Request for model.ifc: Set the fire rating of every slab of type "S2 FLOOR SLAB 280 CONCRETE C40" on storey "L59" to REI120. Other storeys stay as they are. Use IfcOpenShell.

First a look at what the model holds.

```python
import ifcopenshell
import ifcopenshell.util.element

model = ifcopenshell.open("model.ifc")
print(model.schema)
storey = next(s for s in model.by_type("IfcBuildingStorey") if s.Name == "L59")
slabs = [e for e in ifcopenshell.util.element.get_decomposition(storey) if e.is_a("IfcSlab")]
seen = {}
for e in slabs:
    element_type = ifcopenshell.util.element.get_type(e)
    key = (element_type.Name if element_type != e and element_type else None, ifcopenshell.util.element.get_pset(e, "Pset_SlabCommon", "FireRating"))
    seen[key] = seen.get(key, 0) + 1
for (name, value), count in sorted(seen.items(), key=str):
    print(count, "x", name, "|", value)
```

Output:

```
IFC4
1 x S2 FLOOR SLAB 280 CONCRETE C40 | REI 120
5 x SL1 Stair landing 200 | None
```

```python
import ifcopenshell
import ifcopenshell.api.pset
import ifcopenshell.util.element

model = ifcopenshell.open("model.ifc")

storey = next(s for s in model.by_type("IfcBuildingStorey") if s.Name == "L59")
slabs = [e for e in ifcopenshell.util.element.get_decomposition(storey) if e.is_a("IfcSlab")]

count = 0
for e in slabs:
    element_type = ifcopenshell.util.element.get_type(e)
    if element_type in (None, e) or element_type.Name != "S2 FLOOR SLAB 280 CONCRETE C40":
        continue
    found = ifcopenshell.util.element.get_pset(e, "Pset_SlabCommon", should_inherit=False)
    if found:
        pset = model.by_id(found["id"])
        if len(ifcopenshell.util.element.get_elements_by_pset(pset)) > 1:
            pset = ifcopenshell.api.pset.unshare_pset(model, products=[e], pset=pset)[0]
    else:
        pset = ifcopenshell.api.pset.add_pset(model, product=e, name="Pset_SlabCommon")
    ifcopenshell.api.pset.edit_pset(model, pset=pset, properties={"FireRating": "REI120"})
    count += 1

print(count, "slabs updated")

model.write("model_rev.ifc")
```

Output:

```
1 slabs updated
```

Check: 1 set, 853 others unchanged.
